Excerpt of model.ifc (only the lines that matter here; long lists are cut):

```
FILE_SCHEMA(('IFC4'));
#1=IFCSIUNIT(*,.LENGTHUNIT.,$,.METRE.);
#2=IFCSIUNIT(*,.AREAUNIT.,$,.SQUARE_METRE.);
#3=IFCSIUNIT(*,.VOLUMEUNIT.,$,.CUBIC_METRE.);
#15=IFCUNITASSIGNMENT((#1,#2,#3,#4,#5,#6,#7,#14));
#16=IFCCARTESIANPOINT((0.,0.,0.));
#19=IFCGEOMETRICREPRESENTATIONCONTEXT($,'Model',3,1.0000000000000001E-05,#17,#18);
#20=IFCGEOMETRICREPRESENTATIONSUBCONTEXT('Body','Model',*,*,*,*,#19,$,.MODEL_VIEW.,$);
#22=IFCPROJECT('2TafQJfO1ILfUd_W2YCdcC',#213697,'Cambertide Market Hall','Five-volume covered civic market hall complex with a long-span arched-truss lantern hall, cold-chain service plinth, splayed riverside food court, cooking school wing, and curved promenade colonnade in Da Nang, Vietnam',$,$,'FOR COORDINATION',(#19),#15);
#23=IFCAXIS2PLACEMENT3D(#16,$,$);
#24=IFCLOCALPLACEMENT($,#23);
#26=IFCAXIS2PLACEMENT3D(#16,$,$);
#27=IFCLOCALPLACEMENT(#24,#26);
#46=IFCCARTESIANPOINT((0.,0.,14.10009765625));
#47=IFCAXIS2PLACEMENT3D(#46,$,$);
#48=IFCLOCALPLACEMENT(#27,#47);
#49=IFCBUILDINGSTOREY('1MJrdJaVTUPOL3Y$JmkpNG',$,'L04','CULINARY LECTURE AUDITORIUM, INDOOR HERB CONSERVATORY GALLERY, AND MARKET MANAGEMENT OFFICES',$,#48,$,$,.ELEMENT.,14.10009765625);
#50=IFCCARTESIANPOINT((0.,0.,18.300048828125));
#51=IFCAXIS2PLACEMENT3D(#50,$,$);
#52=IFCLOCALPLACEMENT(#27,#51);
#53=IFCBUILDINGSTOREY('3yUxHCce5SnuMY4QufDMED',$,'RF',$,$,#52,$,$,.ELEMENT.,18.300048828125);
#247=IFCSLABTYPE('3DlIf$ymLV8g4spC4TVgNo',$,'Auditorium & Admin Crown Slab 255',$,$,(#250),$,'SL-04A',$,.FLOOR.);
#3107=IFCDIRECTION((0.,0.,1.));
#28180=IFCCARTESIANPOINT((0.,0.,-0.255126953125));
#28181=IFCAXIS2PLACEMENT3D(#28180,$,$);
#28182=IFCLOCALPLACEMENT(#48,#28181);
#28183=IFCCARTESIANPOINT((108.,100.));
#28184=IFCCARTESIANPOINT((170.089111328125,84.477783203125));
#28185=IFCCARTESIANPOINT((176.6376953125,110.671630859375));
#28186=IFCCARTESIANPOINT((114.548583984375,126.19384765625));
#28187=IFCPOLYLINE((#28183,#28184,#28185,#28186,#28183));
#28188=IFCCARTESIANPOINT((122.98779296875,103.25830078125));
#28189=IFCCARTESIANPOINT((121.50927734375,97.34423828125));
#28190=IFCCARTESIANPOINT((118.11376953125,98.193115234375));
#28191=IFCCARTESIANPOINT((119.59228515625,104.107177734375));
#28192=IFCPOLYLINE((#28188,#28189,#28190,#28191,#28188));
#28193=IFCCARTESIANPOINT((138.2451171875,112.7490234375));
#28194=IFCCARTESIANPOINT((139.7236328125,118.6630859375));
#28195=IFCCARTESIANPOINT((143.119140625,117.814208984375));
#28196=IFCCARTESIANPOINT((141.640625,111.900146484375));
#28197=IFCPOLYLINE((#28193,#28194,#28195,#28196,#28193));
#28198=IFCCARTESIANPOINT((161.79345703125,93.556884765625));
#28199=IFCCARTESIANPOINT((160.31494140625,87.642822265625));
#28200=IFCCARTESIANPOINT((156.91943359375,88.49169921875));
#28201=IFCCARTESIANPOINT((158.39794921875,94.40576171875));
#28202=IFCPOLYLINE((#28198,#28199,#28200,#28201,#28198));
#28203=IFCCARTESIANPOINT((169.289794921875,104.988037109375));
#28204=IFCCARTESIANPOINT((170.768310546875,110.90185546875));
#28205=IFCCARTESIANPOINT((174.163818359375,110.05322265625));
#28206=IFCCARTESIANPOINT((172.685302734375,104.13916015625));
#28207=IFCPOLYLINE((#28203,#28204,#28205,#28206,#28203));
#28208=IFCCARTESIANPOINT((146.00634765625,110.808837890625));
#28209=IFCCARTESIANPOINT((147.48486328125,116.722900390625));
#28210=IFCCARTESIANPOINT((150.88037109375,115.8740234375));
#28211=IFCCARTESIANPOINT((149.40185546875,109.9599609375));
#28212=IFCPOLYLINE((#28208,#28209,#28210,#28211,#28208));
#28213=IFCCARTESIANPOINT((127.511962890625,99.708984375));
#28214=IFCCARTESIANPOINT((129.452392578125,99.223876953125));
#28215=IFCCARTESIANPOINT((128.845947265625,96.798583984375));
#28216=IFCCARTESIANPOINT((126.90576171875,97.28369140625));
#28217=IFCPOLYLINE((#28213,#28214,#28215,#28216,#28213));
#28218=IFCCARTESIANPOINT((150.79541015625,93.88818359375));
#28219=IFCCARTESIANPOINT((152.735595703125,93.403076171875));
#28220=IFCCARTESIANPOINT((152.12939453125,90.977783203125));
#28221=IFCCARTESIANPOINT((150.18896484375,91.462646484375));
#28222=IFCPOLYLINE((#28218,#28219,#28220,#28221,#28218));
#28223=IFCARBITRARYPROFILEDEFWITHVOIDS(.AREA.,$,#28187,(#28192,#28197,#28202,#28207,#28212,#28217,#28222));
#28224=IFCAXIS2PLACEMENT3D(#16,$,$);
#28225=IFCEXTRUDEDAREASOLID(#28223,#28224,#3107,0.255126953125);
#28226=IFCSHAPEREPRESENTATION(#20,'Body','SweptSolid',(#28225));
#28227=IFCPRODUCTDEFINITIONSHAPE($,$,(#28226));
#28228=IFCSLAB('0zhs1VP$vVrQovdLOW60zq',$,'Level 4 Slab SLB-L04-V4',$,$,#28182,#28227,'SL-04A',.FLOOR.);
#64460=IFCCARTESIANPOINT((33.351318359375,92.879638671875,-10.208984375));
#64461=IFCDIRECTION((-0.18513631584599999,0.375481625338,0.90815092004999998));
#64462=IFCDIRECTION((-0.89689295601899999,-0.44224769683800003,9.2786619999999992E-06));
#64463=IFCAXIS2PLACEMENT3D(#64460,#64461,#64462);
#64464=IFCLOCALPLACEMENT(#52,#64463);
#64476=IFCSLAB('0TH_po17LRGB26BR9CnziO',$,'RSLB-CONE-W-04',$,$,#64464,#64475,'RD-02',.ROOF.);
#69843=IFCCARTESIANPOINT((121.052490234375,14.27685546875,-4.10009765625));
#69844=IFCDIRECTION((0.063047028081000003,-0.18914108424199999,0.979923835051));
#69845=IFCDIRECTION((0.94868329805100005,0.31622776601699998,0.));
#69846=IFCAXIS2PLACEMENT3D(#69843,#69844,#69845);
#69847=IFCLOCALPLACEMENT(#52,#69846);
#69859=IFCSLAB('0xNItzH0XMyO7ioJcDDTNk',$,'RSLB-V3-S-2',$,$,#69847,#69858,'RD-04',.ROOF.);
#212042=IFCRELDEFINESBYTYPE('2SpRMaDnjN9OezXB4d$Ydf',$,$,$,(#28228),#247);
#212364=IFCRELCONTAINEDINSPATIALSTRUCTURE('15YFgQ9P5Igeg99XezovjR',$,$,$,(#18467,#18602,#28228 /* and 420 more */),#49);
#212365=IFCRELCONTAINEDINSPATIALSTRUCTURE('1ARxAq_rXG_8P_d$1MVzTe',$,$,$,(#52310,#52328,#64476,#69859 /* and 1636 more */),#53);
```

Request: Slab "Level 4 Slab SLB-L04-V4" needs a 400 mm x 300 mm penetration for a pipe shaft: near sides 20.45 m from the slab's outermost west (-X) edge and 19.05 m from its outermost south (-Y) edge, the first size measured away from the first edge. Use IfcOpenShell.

```python
import numpy as np
import ifcopenshell
import ifcopenshell.api.feature
import ifcopenshell.api.geometry
import ifcopenshell.api.root
import ifcopenshell.geom
import ifcopenshell.util.placement
import ifcopenshell.util.representation
import ifcopenshell.util.shape
import ifcopenshell.util.unit

model = ifcopenshell.open("model.ifc")
unit_scale = ifcopenshell.util.unit.calculate_unit_scale(model)
settings = ifcopenshell.geom.settings()


def volume(element):
    """Net volume in cubic metres, openings subtracted."""
    shape = ifcopenshell.geom.create_shape(settings, element)
    return ifcopenshell.util.shape.get_volume(shape.geometry)


slab = model.by_guid("0zhs1VP$vVrQovdLOW60zq")
before = volume(slab)

# Extent in the slab's own axes, in metres. The edges named are its -X and -Y sides.
slab_shape = ifcopenshell.geom.create_shape(settings, slab)
vertices = ifcopenshell.util.shape.get_vertices(slab_shape.geometry)
x_min, y_min, bottom = vertices.min(axis=0)
top = vertices[:, 2].max()

opening = ifcopenshell.api.root.create_entity(model, ifc_class="IfcOpeningElement", name="Pipe shaft opening", predefined_type="OPENING")
context = ifcopenshell.util.representation.get_context(model, "Model", "Body", "MODEL_VIEW")
width, depth = 0.4, 0.3
outline = [(0.0, 0.0), (width, 0.0), (width, depth), (0.0, depth), (0.0, 0.0)]
# Overshoot both faces by 50 mm so the cut is clean.
shape = ifcopenshell.api.geometry.add_slab_representation(
    model, context=context, depth=top - bottom + 0.1, polyline=outline
)
ifcopenshell.api.geometry.assign_representation(model, product=opening, representation=shape)

matrix = ifcopenshell.util.placement.get_local_placement(slab.ObjectPlacement)
matrix[:, 3] = matrix @ np.append(np.array([x_min + 20.45, y_min + 19.05, bottom - 0.05]) / unit_scale, 1.0)
ifcopenshell.api.geometry.edit_object_placement(model, product=opening, matrix=matrix, is_si=False)
ifcopenshell.api.feature.add_feature(model, feature=opening, element=slab)

after = volume(slab)

print(f"slab volume {before:.3f} -> {after:.3f} m3")

model.write("model_rev.ifc")
```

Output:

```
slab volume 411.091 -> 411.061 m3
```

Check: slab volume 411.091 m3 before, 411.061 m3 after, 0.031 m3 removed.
